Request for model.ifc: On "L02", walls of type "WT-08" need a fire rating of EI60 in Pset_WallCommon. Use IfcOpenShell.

First a look at what the model holds.

```python
import ifcopenshell
import ifcopenshell.util.element

model = ifcopenshell.open("model.ifc")
print(model.schema)
storey = next(s for s in model.by_type("IfcBuildingStorey") if s.Name == "L02")
walls = [e for e in ifcopenshell.util.element.get_decomposition(storey) if e.is_a("IfcWall")]
seen = {}
for e in walls:
    element_type = ifcopenshell.util.element.get_type(e)
    key = (element_type.Name if element_type != e and element_type else None, ifcopenshell.util.element.get_pset(e, "Pset_WallCommon", "FireRating"))
    seen[key] = seen.get(key, 0) + 1
for (name, value), count in sorted(seen.items(), key=str):
    print(count, "x", name, "|", value)
```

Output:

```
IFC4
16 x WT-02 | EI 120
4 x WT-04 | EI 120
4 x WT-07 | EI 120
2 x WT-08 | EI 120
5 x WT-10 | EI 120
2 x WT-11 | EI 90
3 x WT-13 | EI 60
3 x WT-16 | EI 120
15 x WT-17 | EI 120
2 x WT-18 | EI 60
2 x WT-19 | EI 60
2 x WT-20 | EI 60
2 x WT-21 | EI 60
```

```python
import ifcopenshell
import ifcopenshell.api.pset
import ifcopenshell.util.element

model = ifcopenshell.open("model.ifc")

storey = next(s for s in model.by_type("IfcBuildingStorey") if s.Name == "L02")
walls = [e for e in ifcopenshell.util.element.get_decomposition(storey) if e.is_a("IfcWall")]

count = 0
for e in walls:
    element_type = ifcopenshell.util.element.get_type(e)
    if element_type in (None, e) or element_type.Name != "WT-08":
        continue
    # add_pset returns the element's existing set when there is one.
    pset = ifcopenshell.api.pset.add_pset(model, product=e, name="Pset_WallCommon")
    ifcopenshell.api.pset.edit_pset(model, pset=pset, properties={"FireRating": "EI60"})
    count += 1

print(count, "walls updated")

model.write("model_updated.ifc")
```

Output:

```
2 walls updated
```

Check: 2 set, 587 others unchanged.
